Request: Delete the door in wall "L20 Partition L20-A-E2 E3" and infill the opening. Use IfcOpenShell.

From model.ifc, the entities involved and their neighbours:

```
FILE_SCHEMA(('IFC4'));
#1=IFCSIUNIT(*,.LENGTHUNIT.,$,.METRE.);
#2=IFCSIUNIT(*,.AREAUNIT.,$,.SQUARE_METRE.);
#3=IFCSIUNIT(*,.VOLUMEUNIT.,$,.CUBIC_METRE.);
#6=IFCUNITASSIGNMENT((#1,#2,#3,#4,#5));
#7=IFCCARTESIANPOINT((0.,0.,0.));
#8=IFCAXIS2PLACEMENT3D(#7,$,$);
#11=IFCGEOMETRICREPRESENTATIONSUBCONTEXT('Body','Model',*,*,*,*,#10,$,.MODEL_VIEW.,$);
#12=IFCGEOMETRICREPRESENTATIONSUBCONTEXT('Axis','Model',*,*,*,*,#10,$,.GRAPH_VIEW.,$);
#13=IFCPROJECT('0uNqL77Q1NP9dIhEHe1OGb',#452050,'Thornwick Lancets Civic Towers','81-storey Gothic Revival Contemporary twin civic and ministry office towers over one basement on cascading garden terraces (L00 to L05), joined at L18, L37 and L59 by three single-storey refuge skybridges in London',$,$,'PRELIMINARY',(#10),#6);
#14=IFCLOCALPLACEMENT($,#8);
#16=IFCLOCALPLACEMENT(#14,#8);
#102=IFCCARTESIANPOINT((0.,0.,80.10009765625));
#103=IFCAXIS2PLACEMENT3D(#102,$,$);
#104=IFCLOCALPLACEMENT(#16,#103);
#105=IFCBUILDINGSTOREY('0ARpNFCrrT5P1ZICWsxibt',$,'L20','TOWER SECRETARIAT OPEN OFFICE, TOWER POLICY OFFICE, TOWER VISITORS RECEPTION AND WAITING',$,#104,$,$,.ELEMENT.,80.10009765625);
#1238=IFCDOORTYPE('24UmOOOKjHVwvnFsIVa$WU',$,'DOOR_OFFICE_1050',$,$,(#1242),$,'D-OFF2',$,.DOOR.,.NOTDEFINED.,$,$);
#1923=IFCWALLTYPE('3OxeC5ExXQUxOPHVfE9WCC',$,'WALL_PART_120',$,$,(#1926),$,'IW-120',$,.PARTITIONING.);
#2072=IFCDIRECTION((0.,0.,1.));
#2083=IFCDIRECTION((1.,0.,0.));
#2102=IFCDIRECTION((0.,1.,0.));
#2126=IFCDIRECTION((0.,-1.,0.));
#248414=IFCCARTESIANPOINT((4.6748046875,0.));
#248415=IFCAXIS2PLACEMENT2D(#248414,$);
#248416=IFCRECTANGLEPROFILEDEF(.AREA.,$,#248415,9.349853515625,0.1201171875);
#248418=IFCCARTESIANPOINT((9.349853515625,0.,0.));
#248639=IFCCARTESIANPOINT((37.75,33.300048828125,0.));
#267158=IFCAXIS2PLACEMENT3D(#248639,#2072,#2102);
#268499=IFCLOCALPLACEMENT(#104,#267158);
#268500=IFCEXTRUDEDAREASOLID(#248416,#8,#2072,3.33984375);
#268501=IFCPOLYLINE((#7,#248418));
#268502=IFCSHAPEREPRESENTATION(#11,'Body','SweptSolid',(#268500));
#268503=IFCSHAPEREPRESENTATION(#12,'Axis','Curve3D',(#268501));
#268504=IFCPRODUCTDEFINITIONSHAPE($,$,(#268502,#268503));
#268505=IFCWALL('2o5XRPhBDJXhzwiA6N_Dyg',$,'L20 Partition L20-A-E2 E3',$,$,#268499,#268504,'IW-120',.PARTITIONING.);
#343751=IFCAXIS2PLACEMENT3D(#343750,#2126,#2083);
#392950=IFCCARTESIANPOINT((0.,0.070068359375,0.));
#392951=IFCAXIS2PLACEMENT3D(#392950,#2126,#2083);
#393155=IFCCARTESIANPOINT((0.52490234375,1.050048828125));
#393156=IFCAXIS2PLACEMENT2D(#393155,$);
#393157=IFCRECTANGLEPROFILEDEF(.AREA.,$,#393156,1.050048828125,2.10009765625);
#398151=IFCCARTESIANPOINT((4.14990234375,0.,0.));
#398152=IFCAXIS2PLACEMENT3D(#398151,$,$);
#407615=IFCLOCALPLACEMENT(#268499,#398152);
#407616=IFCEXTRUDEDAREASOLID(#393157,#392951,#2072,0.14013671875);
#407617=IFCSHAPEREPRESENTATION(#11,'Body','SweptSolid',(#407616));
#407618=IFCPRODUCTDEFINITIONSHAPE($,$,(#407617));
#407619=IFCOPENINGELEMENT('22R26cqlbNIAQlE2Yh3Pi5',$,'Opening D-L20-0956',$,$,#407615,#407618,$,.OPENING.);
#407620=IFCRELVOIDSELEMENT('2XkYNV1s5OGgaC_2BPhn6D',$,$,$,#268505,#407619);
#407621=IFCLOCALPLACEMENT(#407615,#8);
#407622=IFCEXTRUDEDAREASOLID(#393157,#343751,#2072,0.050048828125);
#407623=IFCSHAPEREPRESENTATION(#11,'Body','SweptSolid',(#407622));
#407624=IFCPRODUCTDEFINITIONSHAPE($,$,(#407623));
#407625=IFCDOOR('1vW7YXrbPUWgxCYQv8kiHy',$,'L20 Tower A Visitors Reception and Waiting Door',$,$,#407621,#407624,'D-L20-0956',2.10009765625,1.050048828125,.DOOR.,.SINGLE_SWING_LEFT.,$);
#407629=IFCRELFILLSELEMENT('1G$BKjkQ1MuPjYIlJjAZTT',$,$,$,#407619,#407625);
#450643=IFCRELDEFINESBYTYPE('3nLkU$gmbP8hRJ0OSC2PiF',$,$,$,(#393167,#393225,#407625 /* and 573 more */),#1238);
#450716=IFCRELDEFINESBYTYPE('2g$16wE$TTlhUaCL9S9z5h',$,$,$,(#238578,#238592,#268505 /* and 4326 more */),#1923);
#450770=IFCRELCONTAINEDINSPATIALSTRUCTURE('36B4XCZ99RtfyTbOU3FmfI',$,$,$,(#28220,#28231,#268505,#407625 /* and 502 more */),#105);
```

```python
import ifcopenshell
import ifcopenshell.api.feature
import ifcopenshell.api.root
import ifcopenshell.geom
import ifcopenshell.util.shape

model = ifcopenshell.open("model.ifc")
settings = ifcopenshell.geom.settings()


def volume(element):
    """Net volume in cubic metres, openings subtracted."""
    shape = ifcopenshell.geom.create_shape(settings, element)
    return ifcopenshell.util.shape.get_volume(shape.geometry)


door = model.by_guid("1vW7YXrbPUWgxCYQv8kiHy")
opening = door.FillsVoids[0].RelatingOpeningElement
wall = opening.VoidsElements[0].RelatingBuildingElement
before = volume(wall)

ifcopenshell.api.root.remove_product(model, product=door)
ifcopenshell.api.feature.remove_feature(model, feature=opening)

after = volume(wall)

print(f"wall volume {before:.3f} -> {after:.3f} m3")

model.write("model_v2.ifc")
```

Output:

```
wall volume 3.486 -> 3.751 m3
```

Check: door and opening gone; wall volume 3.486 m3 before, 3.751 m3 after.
